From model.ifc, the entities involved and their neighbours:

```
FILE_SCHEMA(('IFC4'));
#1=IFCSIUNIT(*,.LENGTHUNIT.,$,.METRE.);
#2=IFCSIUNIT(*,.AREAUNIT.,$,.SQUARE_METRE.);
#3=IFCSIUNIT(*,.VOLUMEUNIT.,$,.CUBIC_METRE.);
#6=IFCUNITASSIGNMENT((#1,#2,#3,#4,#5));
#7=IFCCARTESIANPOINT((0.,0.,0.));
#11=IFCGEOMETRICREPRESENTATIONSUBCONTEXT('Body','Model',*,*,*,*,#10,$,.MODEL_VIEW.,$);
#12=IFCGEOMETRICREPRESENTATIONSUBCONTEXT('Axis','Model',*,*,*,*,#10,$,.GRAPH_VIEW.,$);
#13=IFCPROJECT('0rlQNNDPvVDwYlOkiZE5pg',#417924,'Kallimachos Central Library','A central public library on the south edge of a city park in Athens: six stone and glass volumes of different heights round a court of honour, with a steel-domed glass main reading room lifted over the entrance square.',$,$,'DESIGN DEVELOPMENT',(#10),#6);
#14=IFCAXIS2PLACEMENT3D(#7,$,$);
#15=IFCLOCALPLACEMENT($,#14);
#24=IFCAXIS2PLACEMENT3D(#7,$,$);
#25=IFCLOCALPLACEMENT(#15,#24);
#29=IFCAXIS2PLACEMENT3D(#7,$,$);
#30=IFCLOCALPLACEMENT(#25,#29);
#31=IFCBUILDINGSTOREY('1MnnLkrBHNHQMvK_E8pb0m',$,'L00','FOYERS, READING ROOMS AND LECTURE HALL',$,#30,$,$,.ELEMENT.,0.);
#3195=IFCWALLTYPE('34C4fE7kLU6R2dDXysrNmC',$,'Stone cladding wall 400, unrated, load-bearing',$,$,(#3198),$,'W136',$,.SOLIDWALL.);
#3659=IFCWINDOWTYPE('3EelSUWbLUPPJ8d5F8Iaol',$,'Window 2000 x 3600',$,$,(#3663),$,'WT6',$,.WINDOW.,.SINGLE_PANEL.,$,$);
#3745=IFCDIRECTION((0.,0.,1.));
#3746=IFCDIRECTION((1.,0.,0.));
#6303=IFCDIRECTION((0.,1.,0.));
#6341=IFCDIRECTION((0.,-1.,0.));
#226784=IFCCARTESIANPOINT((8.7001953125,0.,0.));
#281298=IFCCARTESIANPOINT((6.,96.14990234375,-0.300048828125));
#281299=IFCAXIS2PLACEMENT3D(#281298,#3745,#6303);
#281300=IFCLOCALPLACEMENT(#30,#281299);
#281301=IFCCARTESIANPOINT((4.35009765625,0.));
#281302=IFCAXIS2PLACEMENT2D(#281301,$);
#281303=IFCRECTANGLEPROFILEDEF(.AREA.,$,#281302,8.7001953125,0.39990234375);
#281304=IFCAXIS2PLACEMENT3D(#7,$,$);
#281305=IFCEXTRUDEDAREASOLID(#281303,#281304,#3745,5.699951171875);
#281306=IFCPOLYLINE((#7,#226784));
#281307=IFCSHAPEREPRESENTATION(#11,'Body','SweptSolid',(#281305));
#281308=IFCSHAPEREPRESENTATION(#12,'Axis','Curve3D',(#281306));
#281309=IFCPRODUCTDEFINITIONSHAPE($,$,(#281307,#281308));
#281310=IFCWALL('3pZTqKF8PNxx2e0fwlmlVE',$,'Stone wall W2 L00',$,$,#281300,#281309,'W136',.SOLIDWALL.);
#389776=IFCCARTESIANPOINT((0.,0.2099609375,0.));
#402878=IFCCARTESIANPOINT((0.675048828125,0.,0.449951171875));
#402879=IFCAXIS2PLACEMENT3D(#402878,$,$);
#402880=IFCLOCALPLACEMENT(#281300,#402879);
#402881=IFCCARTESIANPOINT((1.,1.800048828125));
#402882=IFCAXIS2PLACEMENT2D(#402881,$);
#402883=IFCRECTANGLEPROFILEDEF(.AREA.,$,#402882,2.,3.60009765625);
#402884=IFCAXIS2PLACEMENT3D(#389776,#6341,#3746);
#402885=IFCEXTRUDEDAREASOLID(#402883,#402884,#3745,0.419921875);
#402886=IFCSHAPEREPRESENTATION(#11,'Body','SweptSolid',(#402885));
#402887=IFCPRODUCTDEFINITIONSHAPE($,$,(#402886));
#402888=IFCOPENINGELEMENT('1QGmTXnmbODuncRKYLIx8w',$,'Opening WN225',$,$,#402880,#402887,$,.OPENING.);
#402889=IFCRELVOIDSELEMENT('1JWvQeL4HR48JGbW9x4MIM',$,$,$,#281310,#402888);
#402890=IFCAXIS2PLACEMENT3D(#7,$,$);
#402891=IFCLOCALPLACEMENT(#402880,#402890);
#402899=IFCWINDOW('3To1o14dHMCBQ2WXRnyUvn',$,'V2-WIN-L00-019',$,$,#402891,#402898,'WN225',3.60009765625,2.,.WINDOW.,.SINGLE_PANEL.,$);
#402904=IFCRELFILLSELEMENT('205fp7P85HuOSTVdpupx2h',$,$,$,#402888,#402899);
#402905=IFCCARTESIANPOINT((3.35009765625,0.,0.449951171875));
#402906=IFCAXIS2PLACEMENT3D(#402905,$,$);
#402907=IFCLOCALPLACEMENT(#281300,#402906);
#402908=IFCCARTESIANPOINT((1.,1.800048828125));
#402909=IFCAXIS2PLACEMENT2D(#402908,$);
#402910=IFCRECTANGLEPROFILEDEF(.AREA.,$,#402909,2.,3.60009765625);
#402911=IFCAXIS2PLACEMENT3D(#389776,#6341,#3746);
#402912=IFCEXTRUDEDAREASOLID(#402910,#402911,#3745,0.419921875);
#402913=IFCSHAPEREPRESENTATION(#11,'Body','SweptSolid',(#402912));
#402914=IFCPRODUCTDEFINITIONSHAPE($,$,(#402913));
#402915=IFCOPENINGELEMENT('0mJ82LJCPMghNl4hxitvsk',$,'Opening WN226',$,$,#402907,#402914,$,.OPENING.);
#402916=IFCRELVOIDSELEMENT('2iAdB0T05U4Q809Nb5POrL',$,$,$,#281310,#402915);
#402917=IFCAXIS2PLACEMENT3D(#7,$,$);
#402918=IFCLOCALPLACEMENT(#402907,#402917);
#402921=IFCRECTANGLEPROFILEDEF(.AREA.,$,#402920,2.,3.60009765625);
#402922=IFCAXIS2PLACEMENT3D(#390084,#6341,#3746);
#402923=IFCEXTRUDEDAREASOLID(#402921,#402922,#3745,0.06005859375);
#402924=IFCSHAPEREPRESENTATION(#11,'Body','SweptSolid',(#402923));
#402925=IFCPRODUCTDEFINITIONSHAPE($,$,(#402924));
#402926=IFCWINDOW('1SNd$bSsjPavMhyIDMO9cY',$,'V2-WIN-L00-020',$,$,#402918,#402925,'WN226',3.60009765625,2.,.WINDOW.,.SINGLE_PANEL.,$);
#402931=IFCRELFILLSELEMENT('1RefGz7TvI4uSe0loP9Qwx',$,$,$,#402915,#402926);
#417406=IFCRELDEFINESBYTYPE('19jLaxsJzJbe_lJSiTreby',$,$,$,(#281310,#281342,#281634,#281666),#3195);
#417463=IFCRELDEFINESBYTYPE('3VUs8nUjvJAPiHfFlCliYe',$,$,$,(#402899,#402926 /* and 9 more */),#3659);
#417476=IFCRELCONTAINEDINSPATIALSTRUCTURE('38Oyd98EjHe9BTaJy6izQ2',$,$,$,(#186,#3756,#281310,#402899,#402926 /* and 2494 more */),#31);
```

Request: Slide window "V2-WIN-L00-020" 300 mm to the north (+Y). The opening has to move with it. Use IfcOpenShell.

```python
import ifcopenshell
import ifcopenshell.api.geometry
import ifcopenshell.util.placement
import ifcopenshell.util.unit

model = ifcopenshell.open("model.ifc")
unit_scale = ifcopenshell.util.unit.calculate_unit_scale(model)

window = model.by_guid("1SNd$bSsjPavMhyIDMO9cY")
opening = window.FillsVoids[0].RelatingOpeningElement
wall = opening.VoidsElements[0].RelatingBuildingElement

wall_matrix = ifcopenshell.util.placement.get_local_placement(wall.ObjectPlacement)
shift = wall_matrix[:3, 0] * 0.3 / unit_scale
before = ifcopenshell.util.placement.get_local_placement(window.ObjectPlacement)[:3, 3].copy()

# The window is placed relative to its opening, so it follows when the opening moves.
matrix = ifcopenshell.util.placement.get_local_placement(opening.ObjectPlacement)
matrix[:3, 3] += shift
ifcopenshell.api.geometry.edit_object_placement(
    model, product=opening, matrix=matrix, is_si=False, should_transform_children=True
)

after = ifcopenshell.util.placement.get_local_placement(window.ObjectPlacement)[:3, 3]
print("window moved by", (after - before).round(3) + 0.0)

model.write("model_rev.ifc")
```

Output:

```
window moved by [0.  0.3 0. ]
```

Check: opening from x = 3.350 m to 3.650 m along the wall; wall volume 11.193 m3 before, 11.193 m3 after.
